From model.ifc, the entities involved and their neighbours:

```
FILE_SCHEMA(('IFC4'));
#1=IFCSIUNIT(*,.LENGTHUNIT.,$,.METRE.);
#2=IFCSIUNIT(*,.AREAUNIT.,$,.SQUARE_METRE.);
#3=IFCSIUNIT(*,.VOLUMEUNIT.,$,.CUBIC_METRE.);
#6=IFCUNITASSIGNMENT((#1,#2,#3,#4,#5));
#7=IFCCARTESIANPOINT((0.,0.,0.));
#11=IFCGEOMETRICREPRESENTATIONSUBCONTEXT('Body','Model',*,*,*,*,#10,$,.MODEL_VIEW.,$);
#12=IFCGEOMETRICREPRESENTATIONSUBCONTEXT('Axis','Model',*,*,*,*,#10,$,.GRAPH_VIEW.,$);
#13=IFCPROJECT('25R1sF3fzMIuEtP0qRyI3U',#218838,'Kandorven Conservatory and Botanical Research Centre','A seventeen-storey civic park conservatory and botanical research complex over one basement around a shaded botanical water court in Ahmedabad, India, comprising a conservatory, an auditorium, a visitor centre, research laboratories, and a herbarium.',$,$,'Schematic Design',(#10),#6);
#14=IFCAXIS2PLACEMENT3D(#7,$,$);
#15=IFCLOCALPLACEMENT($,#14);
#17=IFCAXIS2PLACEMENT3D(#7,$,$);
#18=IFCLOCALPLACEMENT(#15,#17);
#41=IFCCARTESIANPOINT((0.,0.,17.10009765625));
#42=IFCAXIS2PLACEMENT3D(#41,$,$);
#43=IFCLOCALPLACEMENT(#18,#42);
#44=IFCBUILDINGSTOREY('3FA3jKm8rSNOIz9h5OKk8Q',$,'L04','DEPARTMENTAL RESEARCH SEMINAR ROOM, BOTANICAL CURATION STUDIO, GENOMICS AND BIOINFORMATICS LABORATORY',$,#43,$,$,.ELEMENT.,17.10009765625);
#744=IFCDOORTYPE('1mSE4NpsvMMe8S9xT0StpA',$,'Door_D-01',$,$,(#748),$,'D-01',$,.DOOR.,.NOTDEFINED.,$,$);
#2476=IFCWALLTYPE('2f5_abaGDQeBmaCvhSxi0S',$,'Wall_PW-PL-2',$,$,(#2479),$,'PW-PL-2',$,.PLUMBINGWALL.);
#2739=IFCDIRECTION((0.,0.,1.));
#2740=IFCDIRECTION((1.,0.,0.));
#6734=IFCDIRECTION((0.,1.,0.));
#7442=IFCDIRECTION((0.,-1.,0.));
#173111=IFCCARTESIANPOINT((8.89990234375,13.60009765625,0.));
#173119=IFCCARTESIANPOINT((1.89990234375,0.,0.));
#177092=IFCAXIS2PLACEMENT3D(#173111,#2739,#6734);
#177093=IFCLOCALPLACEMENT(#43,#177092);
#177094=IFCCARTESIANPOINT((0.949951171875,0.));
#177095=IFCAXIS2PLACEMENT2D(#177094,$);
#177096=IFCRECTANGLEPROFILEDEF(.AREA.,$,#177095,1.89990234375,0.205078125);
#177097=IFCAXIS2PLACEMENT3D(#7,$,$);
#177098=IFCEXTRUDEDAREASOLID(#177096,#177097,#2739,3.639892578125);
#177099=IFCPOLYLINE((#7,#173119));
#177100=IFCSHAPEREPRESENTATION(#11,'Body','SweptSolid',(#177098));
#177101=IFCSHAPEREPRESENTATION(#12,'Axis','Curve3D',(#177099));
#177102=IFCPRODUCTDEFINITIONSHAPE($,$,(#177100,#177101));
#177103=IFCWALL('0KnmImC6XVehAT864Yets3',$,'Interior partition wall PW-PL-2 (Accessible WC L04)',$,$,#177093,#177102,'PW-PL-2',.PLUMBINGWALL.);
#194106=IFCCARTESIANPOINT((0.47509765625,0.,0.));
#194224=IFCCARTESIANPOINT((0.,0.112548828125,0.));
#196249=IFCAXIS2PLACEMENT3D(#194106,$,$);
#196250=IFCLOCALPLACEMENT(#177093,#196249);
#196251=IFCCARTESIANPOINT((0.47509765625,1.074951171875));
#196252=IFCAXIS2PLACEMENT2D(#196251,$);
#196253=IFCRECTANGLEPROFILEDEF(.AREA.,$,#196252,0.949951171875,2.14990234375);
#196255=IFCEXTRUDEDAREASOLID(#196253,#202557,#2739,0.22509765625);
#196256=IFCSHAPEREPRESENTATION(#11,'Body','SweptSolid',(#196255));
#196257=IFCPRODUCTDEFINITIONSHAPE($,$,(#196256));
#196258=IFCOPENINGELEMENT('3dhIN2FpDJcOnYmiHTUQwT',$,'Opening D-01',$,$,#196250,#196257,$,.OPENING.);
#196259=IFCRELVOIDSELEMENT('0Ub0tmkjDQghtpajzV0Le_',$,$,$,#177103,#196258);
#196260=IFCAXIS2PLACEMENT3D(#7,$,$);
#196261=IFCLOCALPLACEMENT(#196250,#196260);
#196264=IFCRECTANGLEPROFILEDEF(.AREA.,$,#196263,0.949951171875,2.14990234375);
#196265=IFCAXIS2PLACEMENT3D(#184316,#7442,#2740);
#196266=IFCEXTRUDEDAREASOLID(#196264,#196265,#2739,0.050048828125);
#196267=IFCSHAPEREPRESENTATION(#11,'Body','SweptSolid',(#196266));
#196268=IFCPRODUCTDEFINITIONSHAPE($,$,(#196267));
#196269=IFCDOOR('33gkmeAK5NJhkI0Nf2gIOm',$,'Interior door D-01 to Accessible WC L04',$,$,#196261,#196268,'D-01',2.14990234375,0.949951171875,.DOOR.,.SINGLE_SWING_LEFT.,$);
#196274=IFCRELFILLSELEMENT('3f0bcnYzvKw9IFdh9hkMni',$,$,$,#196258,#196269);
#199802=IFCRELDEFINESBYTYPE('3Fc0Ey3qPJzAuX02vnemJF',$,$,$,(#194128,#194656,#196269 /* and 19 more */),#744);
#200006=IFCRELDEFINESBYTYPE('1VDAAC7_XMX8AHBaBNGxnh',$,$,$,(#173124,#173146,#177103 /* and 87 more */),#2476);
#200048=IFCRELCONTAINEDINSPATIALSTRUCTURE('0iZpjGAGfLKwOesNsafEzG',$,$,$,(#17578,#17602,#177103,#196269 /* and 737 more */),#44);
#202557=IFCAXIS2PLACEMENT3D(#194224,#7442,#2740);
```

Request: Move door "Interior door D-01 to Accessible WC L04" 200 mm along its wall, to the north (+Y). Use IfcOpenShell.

```python
import ifcopenshell
import ifcopenshell.api.geometry
import ifcopenshell.util.placement
import ifcopenshell.util.unit

model = ifcopenshell.open("model.ifc")
unit_scale = ifcopenshell.util.unit.calculate_unit_scale(model)

door = model.by_guid("33gkmeAK5NJhkI0Nf2gIOm")
opening = door.FillsVoids[0].RelatingOpeningElement
wall = opening.VoidsElements[0].RelatingBuildingElement

wall_matrix = ifcopenshell.util.placement.get_local_placement(wall.ObjectPlacement)
shift = wall_matrix[:3, 0] * 0.2 / unit_scale
before = ifcopenshell.util.placement.get_local_placement(door.ObjectPlacement)[:3, 3].copy()

# The door is placed relative to its opening, so it follows when the opening moves.
matrix = ifcopenshell.util.placement.get_local_placement(opening.ObjectPlacement)
matrix[:3, 3] += shift
ifcopenshell.api.geometry.edit_object_placement(
    model, product=opening, matrix=matrix, is_si=False, should_transform_children=True
)

after = ifcopenshell.util.placement.get_local_placement(door.ObjectPlacement)[:3, 3]
print("door moved by", (after - before).round(3) + 0.0)

model.write("model_updated.ifc")
```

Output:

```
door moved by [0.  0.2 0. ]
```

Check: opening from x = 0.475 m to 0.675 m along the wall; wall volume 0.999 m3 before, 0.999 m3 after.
